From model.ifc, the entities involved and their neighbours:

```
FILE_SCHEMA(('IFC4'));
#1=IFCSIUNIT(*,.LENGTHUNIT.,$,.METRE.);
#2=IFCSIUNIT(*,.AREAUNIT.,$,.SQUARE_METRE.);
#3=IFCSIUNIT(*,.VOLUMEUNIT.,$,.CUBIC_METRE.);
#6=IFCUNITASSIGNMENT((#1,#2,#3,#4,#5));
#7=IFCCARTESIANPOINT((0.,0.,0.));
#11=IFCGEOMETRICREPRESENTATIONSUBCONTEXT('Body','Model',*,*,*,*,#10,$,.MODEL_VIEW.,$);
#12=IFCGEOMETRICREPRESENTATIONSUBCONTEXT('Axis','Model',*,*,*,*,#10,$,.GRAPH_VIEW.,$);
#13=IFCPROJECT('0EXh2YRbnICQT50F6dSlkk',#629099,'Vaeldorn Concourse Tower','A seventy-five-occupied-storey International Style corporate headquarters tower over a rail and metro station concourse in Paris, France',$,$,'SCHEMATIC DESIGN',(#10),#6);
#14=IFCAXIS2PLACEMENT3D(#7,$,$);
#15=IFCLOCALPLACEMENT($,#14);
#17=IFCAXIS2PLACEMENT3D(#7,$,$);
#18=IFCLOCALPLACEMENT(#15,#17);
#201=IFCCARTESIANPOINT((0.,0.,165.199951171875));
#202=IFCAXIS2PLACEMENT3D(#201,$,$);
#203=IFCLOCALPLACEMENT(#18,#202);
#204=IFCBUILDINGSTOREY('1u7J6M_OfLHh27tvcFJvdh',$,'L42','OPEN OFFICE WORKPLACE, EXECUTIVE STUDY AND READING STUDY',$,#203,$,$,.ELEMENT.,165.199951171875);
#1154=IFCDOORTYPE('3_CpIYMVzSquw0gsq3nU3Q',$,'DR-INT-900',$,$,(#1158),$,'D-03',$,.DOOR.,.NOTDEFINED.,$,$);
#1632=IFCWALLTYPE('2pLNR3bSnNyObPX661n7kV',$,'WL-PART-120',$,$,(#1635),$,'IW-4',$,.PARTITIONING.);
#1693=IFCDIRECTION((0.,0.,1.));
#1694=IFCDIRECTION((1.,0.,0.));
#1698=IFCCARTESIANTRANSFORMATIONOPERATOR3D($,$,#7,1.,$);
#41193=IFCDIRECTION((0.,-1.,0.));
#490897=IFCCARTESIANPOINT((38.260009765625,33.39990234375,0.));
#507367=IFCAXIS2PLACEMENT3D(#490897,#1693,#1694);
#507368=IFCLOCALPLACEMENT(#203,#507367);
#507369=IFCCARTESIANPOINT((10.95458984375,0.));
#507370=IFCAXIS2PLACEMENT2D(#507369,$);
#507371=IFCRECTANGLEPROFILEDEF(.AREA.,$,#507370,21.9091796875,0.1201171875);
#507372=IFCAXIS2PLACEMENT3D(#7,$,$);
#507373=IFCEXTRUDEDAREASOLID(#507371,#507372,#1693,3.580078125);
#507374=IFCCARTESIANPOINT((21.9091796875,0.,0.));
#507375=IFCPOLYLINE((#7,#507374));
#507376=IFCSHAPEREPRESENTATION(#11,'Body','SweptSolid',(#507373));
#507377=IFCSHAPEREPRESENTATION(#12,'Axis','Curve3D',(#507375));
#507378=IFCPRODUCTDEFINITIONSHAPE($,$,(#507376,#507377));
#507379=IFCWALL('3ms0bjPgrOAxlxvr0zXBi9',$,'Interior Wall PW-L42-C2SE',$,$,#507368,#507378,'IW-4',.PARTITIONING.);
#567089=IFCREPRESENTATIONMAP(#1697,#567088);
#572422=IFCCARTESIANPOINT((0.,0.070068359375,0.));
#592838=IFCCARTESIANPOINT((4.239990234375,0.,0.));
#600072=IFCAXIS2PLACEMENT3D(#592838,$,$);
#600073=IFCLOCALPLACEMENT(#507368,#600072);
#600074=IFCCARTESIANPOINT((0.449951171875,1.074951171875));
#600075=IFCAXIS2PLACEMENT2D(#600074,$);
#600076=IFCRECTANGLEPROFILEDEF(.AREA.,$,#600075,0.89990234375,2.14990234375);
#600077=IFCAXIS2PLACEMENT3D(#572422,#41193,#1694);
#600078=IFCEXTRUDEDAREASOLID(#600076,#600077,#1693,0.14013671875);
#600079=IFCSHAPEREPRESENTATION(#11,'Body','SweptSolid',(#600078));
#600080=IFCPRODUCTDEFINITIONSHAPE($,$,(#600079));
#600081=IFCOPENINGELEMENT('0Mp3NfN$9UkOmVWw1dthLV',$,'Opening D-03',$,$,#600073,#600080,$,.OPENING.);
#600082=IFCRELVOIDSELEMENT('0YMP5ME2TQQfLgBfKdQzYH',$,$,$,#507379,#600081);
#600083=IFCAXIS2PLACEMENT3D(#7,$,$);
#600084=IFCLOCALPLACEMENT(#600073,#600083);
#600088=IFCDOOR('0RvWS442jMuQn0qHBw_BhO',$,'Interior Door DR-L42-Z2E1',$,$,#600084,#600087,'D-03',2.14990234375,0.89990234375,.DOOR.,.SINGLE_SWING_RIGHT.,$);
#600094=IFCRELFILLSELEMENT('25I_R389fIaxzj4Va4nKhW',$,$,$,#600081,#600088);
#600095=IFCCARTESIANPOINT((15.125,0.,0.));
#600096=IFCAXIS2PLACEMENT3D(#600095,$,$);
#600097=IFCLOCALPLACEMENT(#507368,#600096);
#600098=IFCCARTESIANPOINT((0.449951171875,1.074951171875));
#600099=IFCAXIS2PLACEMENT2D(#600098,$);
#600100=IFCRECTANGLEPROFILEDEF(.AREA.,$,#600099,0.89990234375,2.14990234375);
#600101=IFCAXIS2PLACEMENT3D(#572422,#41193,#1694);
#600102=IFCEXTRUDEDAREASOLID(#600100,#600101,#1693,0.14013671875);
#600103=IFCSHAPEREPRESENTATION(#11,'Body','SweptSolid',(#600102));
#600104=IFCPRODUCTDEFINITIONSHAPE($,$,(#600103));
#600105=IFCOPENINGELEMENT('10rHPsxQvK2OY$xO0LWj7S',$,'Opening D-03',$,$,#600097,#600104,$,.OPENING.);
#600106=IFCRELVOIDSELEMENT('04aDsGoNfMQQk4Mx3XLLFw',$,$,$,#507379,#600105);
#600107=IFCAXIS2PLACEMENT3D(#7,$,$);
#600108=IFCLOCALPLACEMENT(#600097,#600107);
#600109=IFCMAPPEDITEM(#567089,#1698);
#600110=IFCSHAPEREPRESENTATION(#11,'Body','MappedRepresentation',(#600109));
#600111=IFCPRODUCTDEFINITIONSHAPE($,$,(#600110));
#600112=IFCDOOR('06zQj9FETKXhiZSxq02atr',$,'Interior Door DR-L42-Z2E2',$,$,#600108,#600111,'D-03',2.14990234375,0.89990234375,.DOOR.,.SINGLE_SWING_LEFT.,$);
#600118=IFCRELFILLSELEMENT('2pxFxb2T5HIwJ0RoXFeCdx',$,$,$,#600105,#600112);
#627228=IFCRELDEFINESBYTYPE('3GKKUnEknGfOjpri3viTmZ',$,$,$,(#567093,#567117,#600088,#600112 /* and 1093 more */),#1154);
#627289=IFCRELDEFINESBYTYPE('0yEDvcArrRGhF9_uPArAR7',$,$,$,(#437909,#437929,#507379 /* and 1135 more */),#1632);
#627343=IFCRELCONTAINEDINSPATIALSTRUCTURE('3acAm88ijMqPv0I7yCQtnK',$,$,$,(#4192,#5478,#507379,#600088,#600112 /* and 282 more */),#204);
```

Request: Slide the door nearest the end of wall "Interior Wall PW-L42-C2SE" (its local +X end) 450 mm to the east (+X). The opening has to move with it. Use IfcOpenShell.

```python
import ifcopenshell
import ifcopenshell.api.geometry
import ifcopenshell.util.placement
import ifcopenshell.util.unit

model = ifcopenshell.open("model.ifc")
unit_scale = ifcopenshell.util.unit.calculate_unit_scale(model)

door = model.by_id(600112)
opening = door.FillsVoids[0].RelatingOpeningElement
wall = opening.VoidsElements[0].RelatingBuildingElement

wall_matrix = ifcopenshell.util.placement.get_local_placement(wall.ObjectPlacement)
shift = wall_matrix[:3, 0] * 0.45 / unit_scale
before = ifcopenshell.util.placement.get_local_placement(door.ObjectPlacement)[:3, 3].copy()

# The door is placed relative to its opening, so it follows when the opening moves.
matrix = ifcopenshell.util.placement.get_local_placement(opening.ObjectPlacement)
matrix[:3, 3] += shift
ifcopenshell.api.geometry.edit_object_placement(
    model, product=opening, matrix=matrix, is_si=False, should_transform_children=True
)

after = ifcopenshell.util.placement.get_local_placement(door.ObjectPlacement)[:3, 3]
print("door moved by", (after - before).round(3) + 0.0)

model.write("model-out.ifc")
```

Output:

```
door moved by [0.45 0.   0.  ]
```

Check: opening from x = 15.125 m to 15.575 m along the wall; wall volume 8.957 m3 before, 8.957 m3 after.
